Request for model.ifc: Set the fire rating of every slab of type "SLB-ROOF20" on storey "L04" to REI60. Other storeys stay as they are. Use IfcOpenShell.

First a look at what the model holds.

```python
import ifcopenshell
import ifcopenshell.util.element

model = ifcopenshell.open("model.ifc")
print(model.schema)
storey = next(s for s in model.by_type("IfcBuildingStorey") if s.Name == "L04")
slabs = [e for e in ifcopenshell.util.element.get_decomposition(storey) if e.is_a("IfcSlab")]
seen = {}
for e in slabs:
    element_type = ifcopenshell.util.element.get_type(e)
    key = (element_type.Name if element_type != e and element_type else None, ifcopenshell.util.element.get_pset(e, "Pset_SlabCommon", "FireRating"))
    seen[key] = seen.get(key, 0) + 1
for (name, value), count in sorted(seen.items(), key=str):
    print(count, "x", name, "|", value)
```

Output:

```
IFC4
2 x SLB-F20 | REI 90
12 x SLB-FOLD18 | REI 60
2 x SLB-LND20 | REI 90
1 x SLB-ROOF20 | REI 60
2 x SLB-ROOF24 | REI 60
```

```python
import ifcopenshell
import ifcopenshell.api.pset
import ifcopenshell.util.element

model = ifcopenshell.open("model.ifc")

storey = next(s for s in model.by_type("IfcBuildingStorey") if s.Name == "L04")
slabs = [e for e in ifcopenshell.util.element.get_decomposition(storey) if e.is_a("IfcSlab")]

count = 0
for e in slabs:
    element_type = ifcopenshell.util.element.get_type(e)
    if element_type in (None, e) or element_type.Name != "SLB-ROOF20":
        continue
    # add_pset returns the element's existing set when there is one.
    pset = ifcopenshell.api.pset.add_pset(model, product=e, name="Pset_SlabCommon")
    ifcopenshell.api.pset.edit_pset(model, pset=pset, properties={"FireRating": "REI60"})
    count += 1

print(count, "slabs updated")

model.write("model-out.ifc")
```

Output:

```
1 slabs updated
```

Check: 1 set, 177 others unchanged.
